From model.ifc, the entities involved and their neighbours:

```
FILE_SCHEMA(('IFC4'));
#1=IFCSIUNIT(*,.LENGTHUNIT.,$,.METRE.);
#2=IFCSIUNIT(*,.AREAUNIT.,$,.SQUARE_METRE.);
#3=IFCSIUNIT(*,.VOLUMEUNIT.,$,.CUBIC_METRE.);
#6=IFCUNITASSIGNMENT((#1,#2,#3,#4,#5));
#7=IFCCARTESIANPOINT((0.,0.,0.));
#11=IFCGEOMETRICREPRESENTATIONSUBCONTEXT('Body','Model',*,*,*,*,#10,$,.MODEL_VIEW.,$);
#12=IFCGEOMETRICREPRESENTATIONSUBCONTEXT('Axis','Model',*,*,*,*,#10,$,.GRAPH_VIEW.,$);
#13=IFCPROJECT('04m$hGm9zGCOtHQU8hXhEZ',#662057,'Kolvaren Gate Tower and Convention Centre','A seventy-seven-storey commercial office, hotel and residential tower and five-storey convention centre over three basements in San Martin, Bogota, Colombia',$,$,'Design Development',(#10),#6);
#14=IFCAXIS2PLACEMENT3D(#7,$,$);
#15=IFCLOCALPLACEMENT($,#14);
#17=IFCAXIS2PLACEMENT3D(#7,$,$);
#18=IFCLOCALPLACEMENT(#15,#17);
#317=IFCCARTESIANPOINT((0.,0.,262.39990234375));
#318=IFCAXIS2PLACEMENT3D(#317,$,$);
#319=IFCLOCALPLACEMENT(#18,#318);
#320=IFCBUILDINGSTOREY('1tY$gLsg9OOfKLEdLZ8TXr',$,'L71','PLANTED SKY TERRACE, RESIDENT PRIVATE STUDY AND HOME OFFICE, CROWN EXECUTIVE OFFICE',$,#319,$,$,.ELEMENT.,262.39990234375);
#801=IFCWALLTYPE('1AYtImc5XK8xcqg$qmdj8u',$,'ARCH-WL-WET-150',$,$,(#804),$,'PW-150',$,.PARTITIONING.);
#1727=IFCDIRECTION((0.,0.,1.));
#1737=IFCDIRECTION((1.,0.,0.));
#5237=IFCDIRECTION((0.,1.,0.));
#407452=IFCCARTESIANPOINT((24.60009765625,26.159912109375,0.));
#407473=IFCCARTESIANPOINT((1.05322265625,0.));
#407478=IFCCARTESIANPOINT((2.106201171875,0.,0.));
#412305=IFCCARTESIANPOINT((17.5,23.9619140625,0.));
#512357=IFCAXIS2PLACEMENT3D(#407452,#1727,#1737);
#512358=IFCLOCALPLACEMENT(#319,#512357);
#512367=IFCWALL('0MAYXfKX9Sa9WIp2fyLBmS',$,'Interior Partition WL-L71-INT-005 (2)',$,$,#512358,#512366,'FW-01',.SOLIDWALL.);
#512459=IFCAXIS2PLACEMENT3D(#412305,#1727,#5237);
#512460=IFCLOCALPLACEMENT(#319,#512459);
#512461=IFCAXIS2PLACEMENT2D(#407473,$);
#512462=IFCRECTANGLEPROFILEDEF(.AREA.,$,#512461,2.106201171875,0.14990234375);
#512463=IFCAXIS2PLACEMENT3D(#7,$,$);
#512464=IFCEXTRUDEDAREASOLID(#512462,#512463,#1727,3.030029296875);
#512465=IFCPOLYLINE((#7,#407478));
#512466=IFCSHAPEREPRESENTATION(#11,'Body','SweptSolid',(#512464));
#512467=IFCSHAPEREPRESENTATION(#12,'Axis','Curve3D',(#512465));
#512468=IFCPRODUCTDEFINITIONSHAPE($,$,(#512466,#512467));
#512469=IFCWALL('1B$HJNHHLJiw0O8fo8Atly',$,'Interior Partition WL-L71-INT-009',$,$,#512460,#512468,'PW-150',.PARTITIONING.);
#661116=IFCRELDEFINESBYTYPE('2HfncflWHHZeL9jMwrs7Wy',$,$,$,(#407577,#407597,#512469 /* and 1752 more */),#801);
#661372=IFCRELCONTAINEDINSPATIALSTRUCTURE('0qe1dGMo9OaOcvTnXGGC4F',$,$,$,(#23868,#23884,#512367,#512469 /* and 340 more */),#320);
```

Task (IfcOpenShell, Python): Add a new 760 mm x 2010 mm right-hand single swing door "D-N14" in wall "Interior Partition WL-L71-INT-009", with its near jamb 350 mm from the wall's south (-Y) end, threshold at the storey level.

```python
import numpy as np
import ifcopenshell
import ifcopenshell.api.feature
import ifcopenshell.api.geometry
import ifcopenshell.api.root
import ifcopenshell.api.spatial
import ifcopenshell.geom
import ifcopenshell.util.element
import ifcopenshell.util.placement
import ifcopenshell.util.representation
import ifcopenshell.util.shape
import ifcopenshell.util.unit

model = ifcopenshell.open("model.ifc")
unit_scale = ifcopenshell.util.unit.calculate_unit_scale(model)
settings = ifcopenshell.geom.settings()


def volume(element):
    """Net volume in cubic metres, openings subtracted."""
    shape = ifcopenshell.geom.create_shape(settings, element)
    return ifcopenshell.util.shape.get_volume(shape.geometry)


wall = model.by_guid("1B$HJNHHLJiw0O8fo8Atly")
storey = ifcopenshell.util.element.get_container(wall, ifc_class="IfcBuildingStorey")
context = ifcopenshell.util.representation.get_context(model, "Model", "Body", "MODEL_VIEW")
before = volume(wall)

width, height, from_end, sill = 0.76, 2.01, 0.35, 0.0  # metres

# The wall runs along its own X axis, and the end named is its -X end.
wall_shape = ifcopenshell.geom.create_shape(settings, wall)
x, y, z = ifcopenshell.util.shape.get_vertices(wall_shape.geometry).T
start = x.min() + from_end
face, thickness = float(y.min()), float(y.max() - y.min())
wall_matrix = ifcopenshell.util.placement.get_local_placement(wall.ObjectPlacement)
level = ifcopenshell.util.placement.get_local_placement(storey.ObjectPlacement)[2, 3]


def in_wall(x, y):
    """Placement at x, y metres in the wall's axes, at sill height."""
    matrix = wall_matrix.copy()
    matrix[:, 3] = wall_matrix @ np.array([x / unit_scale, y / unit_scale, 0.0, 1.0])
    matrix[2, 3] = level + sill / unit_scale
    return matrix


# Opening: a box that overshoots both wall faces by 50 mm.
opening = ifcopenshell.api.root.create_entity(model, ifc_class="IfcOpeningElement", predefined_type="OPENING")
box = ifcopenshell.api.geometry.add_wall_representation(
    model, context=context, length=width, height=height, thickness=thickness + 0.1
)
ifcopenshell.api.geometry.assign_representation(model, product=opening, representation=box)
ifcopenshell.api.geometry.edit_object_placement(model, product=opening, matrix=in_wall(start, face - 0.05), is_si=False)
ifcopenshell.api.feature.add_feature(model, feature=opening, element=wall)

door = ifcopenshell.api.root.create_entity(model, ifc_class="IfcDoor", name="D-N14", predefined_type="DOOR")
door.OverallWidth, door.OverallHeight = width / unit_scale, height / unit_scale
door.OperationType = "SINGLE_SWING_RIGHT"
body = ifcopenshell.api.geometry.add_door_representation(
    model,
    context=context,
    overall_width=door.OverallWidth,
    overall_height=door.OverallHeight,
    operation_type="SINGLE_SWING_RIGHT",
    lining_properties={"LiningDepth": thickness / unit_scale, "ThresholdDepth": thickness / unit_scale},
)
ifcopenshell.api.geometry.assign_representation(model, product=door, representation=body)
ifcopenshell.api.spatial.assign_container(model, products=[door], relating_structure=storey)
ifcopenshell.api.feature.add_filling(model, opening=opening, element=door)

# The lining spans the wall, so the door starts at the wall face.
ifcopenshell.api.geometry.edit_object_placement(model, product=door, matrix=in_wall(start, face), is_si=False)

after = volume(wall)

print(f"wall volume {before:.3f} -> {after:.3f} m3")

model.write("model_rev.ifc")
```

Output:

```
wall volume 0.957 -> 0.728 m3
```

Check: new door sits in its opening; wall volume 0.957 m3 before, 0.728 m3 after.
